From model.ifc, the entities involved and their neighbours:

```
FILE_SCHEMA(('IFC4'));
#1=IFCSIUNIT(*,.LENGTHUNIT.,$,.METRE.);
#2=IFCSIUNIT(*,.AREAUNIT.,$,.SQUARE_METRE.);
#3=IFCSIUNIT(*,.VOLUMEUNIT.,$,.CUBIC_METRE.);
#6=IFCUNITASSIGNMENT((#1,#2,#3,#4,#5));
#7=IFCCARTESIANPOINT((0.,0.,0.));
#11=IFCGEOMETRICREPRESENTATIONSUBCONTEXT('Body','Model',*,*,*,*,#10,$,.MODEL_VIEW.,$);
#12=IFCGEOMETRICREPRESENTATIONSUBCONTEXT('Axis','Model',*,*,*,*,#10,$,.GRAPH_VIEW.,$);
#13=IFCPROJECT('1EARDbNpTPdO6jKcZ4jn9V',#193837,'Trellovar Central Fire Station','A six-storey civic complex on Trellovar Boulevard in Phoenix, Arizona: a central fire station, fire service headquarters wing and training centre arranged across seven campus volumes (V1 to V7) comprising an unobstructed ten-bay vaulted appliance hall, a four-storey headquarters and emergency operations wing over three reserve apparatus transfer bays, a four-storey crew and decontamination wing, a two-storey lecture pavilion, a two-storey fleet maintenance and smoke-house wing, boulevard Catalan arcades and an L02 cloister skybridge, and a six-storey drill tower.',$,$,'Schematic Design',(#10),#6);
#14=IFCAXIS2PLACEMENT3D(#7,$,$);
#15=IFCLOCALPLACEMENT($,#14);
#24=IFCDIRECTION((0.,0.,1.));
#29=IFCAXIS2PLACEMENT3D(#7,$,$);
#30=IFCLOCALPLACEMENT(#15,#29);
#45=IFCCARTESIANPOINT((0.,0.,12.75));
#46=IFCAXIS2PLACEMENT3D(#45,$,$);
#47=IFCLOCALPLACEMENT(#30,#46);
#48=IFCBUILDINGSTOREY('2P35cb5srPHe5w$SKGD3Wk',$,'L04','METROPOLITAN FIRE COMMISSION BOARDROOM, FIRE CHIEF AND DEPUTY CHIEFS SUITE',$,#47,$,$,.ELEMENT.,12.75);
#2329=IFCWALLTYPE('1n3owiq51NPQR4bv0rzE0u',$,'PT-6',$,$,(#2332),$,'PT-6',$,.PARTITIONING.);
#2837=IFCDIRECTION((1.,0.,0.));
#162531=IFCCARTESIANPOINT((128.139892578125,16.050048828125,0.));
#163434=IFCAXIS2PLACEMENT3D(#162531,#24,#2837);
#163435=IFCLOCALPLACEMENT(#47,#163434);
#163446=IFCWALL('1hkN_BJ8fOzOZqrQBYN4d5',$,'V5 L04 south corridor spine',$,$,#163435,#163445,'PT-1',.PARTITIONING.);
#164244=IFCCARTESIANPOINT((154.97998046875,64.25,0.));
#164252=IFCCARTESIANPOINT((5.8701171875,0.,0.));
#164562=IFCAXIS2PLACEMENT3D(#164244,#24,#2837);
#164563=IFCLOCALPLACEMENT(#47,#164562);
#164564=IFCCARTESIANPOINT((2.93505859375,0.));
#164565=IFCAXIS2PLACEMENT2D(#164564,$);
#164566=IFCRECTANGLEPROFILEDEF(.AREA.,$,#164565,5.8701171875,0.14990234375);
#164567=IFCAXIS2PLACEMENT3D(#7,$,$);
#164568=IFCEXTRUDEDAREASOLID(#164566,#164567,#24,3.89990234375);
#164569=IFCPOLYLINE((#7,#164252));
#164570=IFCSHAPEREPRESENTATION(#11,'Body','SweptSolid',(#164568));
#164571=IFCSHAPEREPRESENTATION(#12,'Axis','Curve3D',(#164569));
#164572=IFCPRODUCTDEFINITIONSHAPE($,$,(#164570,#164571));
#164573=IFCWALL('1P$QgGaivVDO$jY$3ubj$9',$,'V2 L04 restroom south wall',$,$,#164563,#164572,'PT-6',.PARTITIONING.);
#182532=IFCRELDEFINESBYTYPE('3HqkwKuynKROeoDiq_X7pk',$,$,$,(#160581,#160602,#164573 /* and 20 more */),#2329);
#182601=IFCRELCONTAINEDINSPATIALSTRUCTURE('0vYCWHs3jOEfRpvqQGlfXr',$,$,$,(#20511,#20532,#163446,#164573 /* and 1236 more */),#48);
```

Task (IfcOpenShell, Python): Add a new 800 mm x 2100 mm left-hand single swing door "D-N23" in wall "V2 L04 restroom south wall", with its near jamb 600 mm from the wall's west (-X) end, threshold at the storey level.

```python
import numpy as np
import ifcopenshell
import ifcopenshell.api.feature
import ifcopenshell.api.geometry
import ifcopenshell.api.root
import ifcopenshell.api.spatial
import ifcopenshell.geom
import ifcopenshell.util.element
import ifcopenshell.util.placement
import ifcopenshell.util.representation
import ifcopenshell.util.shape
import ifcopenshell.util.unit

model = ifcopenshell.open("model.ifc")
unit_scale = ifcopenshell.util.unit.calculate_unit_scale(model)
settings = ifcopenshell.geom.settings()


def volume(element):
    """Net volume in cubic metres, openings subtracted."""
    shape = ifcopenshell.geom.create_shape(settings, element)
    return ifcopenshell.util.shape.get_volume(shape.geometry)


wall = model.by_guid("1P$QgGaivVDO$jY$3ubj$9")
storey = ifcopenshell.util.element.get_container(wall, ifc_class="IfcBuildingStorey")
context = ifcopenshell.util.representation.get_context(model, "Model", "Body", "MODEL_VIEW")
before = volume(wall)

width, height, from_end, sill = 0.8, 2.1, 0.6, 0.0  # metres

# The wall runs along its own X axis, and the end named is its -X end.
wall_shape = ifcopenshell.geom.create_shape(settings, wall)
x, y, z = ifcopenshell.util.shape.get_vertices(wall_shape.geometry).T
start = x.min() + from_end
face, thickness = float(y.min()), float(y.max() - y.min())
wall_matrix = ifcopenshell.util.placement.get_local_placement(wall.ObjectPlacement)
level = ifcopenshell.util.placement.get_local_placement(storey.ObjectPlacement)[2, 3]


def in_wall(x, y):
    """Placement at x, y metres in the wall's axes, at sill height."""
    matrix = wall_matrix.copy()
    matrix[:, 3] = wall_matrix @ np.array([x / unit_scale, y / unit_scale, 0.0, 1.0])
    matrix[2, 3] = level + sill / unit_scale
    return matrix


# Opening: a box that overshoots both wall faces by 50 mm.
opening = ifcopenshell.api.root.create_entity(model, ifc_class="IfcOpeningElement", predefined_type="OPENING")
box = ifcopenshell.api.geometry.add_wall_representation(
    model, context=context, length=width, height=height, thickness=thickness + 0.1
)
ifcopenshell.api.geometry.assign_representation(model, product=opening, representation=box)
ifcopenshell.api.geometry.edit_object_placement(model, product=opening, matrix=in_wall(start, face - 0.05), is_si=False)
ifcopenshell.api.feature.add_feature(model, feature=opening, element=wall)

door = ifcopenshell.api.root.create_entity(model, ifc_class="IfcDoor", name="D-N23", predefined_type="DOOR")
door.OverallWidth, door.OverallHeight = width / unit_scale, height / unit_scale
door.OperationType = "SINGLE_SWING_LEFT"
body = ifcopenshell.api.geometry.add_door_representation(
    model,
    context=context,
    overall_width=door.OverallWidth,
    overall_height=door.OverallHeight,
    operation_type="SINGLE_SWING_LEFT",
    lining_properties={"LiningDepth": thickness / unit_scale, "ThresholdDepth": thickness / unit_scale},
)
ifcopenshell.api.geometry.assign_representation(model, product=door, representation=body)
ifcopenshell.api.spatial.assign_container(model, products=[door], relating_structure=storey)
ifcopenshell.api.feature.add_filling(model, opening=opening, element=door)

# The lining spans the wall, so the door starts at the wall face.
ifcopenshell.api.geometry.edit_object_placement(model, product=door, matrix=in_wall(start, face), is_si=False)

after = volume(wall)

print(f"wall volume {before:.3f} -> {after:.3f} m3")

model.write("model_updated.ifc")
```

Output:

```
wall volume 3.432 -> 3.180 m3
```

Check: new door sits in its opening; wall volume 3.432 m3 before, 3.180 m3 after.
